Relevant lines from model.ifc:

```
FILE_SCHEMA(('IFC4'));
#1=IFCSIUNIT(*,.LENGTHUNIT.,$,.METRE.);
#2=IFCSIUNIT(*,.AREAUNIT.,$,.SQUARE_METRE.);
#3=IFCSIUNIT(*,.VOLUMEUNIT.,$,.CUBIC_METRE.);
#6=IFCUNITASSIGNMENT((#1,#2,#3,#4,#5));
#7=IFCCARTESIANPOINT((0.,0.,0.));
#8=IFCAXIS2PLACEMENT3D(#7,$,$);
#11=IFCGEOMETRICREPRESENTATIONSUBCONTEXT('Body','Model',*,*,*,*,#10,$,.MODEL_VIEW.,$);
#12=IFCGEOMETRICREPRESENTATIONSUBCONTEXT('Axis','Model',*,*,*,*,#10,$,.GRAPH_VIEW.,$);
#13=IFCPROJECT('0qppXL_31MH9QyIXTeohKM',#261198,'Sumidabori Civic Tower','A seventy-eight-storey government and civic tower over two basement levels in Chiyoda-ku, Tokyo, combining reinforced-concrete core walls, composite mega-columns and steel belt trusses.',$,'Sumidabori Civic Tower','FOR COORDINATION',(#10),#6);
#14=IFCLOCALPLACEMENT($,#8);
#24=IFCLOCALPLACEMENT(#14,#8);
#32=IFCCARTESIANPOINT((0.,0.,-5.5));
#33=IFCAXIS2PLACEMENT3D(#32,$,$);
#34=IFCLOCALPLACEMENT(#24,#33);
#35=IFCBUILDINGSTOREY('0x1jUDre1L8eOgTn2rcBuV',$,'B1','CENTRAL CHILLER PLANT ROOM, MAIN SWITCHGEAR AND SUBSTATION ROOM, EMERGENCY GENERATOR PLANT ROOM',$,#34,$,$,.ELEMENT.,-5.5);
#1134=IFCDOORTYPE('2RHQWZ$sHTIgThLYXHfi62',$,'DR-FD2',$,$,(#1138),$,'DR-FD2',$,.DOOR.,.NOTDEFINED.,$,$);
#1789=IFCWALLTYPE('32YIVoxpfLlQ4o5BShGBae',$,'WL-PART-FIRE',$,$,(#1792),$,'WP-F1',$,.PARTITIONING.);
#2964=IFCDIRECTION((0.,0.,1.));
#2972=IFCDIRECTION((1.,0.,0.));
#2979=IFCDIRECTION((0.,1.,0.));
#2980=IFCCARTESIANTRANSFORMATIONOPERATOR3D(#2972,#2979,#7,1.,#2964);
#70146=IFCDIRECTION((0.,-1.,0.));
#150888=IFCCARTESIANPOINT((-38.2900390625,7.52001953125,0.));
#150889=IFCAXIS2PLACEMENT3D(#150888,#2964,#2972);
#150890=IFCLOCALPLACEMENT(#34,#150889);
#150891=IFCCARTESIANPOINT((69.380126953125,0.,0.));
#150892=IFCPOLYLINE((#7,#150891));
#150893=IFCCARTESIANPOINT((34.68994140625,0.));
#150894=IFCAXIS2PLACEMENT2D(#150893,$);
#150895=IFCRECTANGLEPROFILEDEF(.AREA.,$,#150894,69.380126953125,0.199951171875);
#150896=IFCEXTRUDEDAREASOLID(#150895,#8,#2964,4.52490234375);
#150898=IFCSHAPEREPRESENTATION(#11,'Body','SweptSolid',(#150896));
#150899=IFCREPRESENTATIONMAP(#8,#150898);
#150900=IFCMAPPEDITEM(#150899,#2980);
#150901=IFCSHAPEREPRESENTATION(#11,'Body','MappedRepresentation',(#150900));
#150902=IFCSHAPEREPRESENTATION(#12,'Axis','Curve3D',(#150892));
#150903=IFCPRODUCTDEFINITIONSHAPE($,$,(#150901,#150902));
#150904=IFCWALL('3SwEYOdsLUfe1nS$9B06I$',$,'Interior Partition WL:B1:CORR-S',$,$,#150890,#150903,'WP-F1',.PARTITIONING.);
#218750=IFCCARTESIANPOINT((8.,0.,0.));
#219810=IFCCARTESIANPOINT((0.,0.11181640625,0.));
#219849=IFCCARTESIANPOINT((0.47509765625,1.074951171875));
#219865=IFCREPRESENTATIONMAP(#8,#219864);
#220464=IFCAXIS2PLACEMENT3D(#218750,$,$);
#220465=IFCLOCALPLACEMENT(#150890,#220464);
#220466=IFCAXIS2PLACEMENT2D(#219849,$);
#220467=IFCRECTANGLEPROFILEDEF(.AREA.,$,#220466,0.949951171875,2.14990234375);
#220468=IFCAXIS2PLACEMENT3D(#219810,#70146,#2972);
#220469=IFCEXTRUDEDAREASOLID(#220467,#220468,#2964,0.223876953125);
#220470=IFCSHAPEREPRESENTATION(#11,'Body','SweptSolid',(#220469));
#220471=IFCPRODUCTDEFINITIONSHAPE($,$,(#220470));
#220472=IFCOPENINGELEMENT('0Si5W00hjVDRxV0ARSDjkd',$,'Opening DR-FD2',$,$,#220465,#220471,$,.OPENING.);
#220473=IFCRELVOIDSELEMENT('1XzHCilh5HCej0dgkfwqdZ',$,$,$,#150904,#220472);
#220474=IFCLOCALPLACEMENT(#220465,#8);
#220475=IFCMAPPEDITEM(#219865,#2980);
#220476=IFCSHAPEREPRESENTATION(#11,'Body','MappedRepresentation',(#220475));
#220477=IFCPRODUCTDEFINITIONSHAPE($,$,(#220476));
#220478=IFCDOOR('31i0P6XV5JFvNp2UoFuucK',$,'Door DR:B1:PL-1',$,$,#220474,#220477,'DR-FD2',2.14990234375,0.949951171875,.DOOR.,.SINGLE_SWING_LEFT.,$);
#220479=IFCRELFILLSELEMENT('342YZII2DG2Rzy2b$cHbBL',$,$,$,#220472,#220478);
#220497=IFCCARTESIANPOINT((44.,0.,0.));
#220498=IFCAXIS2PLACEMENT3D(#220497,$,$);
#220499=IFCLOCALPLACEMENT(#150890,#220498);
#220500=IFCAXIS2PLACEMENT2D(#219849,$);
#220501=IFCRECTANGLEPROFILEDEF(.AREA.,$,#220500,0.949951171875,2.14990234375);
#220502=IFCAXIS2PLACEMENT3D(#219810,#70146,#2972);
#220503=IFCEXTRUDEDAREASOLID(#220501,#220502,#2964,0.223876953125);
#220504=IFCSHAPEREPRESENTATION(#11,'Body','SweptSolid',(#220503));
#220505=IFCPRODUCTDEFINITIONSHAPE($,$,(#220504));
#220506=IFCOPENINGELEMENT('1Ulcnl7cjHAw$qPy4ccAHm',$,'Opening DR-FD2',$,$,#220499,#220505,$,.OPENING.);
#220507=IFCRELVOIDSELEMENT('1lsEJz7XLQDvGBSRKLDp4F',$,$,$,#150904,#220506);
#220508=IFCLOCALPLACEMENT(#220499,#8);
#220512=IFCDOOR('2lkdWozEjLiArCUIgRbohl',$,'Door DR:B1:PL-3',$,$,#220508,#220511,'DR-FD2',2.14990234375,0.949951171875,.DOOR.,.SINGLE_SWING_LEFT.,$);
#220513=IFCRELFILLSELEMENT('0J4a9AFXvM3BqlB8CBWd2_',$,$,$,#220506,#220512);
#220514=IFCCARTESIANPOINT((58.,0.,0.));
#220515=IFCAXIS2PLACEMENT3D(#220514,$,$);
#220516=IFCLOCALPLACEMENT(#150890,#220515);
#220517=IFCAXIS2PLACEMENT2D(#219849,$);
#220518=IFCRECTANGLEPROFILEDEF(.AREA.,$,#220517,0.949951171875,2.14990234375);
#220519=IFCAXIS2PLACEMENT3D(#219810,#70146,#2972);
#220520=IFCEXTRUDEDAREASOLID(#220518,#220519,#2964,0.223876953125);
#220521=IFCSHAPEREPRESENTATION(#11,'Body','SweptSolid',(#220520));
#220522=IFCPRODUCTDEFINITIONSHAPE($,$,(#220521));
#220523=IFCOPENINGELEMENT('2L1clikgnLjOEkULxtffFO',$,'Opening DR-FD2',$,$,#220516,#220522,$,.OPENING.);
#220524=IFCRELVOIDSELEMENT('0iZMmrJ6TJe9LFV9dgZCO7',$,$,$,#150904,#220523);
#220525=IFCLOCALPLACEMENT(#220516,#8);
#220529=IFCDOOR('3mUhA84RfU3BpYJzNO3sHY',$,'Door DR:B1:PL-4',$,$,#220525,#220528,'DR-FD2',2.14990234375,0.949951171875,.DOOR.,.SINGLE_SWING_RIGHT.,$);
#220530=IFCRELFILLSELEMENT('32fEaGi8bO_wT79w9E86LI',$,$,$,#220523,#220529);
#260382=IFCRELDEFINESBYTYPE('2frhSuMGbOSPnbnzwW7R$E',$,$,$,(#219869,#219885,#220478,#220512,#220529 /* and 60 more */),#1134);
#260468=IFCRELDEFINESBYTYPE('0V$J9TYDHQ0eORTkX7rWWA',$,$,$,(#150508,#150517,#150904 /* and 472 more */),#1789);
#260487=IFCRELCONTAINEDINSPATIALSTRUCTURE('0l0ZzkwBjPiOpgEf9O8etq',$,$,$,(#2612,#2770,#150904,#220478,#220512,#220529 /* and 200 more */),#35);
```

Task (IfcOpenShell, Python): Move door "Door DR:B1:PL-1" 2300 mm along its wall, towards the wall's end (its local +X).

```python
import ifcopenshell
import ifcopenshell.api.geometry
import ifcopenshell.util.placement
import ifcopenshell.util.unit

model = ifcopenshell.open("model.ifc")
unit_scale = ifcopenshell.util.unit.calculate_unit_scale(model)

door = model.by_id(220478)
opening = door.FillsVoids[0].RelatingOpeningElement
wall = opening.VoidsElements[0].RelatingBuildingElement

wall_matrix = ifcopenshell.util.placement.get_local_placement(wall.ObjectPlacement)
shift = wall_matrix[:3, 0] * 2.3 / unit_scale
before = ifcopenshell.util.placement.get_local_placement(door.ObjectPlacement)[:3, 3].copy()

# The door is placed relative to its opening, so it follows when the opening moves.
matrix = ifcopenshell.util.placement.get_local_placement(opening.ObjectPlacement)
matrix[:3, 3] += shift
ifcopenshell.api.geometry.edit_object_placement(
    model, product=opening, matrix=matrix, is_si=False, should_transform_children=True
)

after = ifcopenshell.util.placement.get_local_placement(door.ObjectPlacement)[:3, 3]
print("door moved by", (after - before).round(3) + 0.0)

model.write("model_updated.ifc")
```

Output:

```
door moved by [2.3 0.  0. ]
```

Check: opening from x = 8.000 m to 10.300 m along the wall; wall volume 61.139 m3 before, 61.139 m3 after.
